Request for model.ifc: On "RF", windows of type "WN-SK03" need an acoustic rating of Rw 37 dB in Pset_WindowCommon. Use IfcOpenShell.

First a look at what the model holds.

```python
import ifcopenshell
import ifcopenshell.util.element

model = ifcopenshell.open("model.ifc")
print(model.schema)
storey = next(s for s in model.by_type("IfcBuildingStorey") if s.Name == "RF")
windows = [e for e in ifcopenshell.util.element.get_decomposition(storey) if e.is_a("IfcWindow")]
seen = {}
for e in windows:
    element_type = ifcopenshell.util.element.get_type(e)
    key = (element_type.Name if element_type != e and element_type else None, ifcopenshell.util.element.get_pset(e, "Pset_WindowCommon", "AcousticRating"))
    seen[key] = seen.get(key, 0) + 1
for (name, value), count in sorted(seen.items(), key=str):
    print(count, "x", name, "|", value)
```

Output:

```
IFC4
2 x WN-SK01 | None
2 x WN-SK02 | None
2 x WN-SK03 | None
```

```python
import ifcopenshell
import ifcopenshell.api.pset
import ifcopenshell.util.element

model = ifcopenshell.open("model.ifc")

storey = next(s for s in model.by_type("IfcBuildingStorey") if s.Name == "RF")
windows = [e for e in ifcopenshell.util.element.get_decomposition(storey) if e.is_a("IfcWindow")]

count = 0
for e in windows:
    element_type = ifcopenshell.util.element.get_type(e)
    if element_type in (None, e) or element_type.Name != "WN-SK03":
        continue
    # add_pset returns the element's existing set when there is one.
    pset = ifcopenshell.api.pset.add_pset(model, product=e, name="Pset_WindowCommon")
    ifcopenshell.api.pset.edit_pset(model, pset=pset, properties={"AcousticRating": "Rw 37 dB"})
    count += 1

print(count, "windows updated")

model.write("model_edited.ifc")
```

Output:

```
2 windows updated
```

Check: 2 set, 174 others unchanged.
